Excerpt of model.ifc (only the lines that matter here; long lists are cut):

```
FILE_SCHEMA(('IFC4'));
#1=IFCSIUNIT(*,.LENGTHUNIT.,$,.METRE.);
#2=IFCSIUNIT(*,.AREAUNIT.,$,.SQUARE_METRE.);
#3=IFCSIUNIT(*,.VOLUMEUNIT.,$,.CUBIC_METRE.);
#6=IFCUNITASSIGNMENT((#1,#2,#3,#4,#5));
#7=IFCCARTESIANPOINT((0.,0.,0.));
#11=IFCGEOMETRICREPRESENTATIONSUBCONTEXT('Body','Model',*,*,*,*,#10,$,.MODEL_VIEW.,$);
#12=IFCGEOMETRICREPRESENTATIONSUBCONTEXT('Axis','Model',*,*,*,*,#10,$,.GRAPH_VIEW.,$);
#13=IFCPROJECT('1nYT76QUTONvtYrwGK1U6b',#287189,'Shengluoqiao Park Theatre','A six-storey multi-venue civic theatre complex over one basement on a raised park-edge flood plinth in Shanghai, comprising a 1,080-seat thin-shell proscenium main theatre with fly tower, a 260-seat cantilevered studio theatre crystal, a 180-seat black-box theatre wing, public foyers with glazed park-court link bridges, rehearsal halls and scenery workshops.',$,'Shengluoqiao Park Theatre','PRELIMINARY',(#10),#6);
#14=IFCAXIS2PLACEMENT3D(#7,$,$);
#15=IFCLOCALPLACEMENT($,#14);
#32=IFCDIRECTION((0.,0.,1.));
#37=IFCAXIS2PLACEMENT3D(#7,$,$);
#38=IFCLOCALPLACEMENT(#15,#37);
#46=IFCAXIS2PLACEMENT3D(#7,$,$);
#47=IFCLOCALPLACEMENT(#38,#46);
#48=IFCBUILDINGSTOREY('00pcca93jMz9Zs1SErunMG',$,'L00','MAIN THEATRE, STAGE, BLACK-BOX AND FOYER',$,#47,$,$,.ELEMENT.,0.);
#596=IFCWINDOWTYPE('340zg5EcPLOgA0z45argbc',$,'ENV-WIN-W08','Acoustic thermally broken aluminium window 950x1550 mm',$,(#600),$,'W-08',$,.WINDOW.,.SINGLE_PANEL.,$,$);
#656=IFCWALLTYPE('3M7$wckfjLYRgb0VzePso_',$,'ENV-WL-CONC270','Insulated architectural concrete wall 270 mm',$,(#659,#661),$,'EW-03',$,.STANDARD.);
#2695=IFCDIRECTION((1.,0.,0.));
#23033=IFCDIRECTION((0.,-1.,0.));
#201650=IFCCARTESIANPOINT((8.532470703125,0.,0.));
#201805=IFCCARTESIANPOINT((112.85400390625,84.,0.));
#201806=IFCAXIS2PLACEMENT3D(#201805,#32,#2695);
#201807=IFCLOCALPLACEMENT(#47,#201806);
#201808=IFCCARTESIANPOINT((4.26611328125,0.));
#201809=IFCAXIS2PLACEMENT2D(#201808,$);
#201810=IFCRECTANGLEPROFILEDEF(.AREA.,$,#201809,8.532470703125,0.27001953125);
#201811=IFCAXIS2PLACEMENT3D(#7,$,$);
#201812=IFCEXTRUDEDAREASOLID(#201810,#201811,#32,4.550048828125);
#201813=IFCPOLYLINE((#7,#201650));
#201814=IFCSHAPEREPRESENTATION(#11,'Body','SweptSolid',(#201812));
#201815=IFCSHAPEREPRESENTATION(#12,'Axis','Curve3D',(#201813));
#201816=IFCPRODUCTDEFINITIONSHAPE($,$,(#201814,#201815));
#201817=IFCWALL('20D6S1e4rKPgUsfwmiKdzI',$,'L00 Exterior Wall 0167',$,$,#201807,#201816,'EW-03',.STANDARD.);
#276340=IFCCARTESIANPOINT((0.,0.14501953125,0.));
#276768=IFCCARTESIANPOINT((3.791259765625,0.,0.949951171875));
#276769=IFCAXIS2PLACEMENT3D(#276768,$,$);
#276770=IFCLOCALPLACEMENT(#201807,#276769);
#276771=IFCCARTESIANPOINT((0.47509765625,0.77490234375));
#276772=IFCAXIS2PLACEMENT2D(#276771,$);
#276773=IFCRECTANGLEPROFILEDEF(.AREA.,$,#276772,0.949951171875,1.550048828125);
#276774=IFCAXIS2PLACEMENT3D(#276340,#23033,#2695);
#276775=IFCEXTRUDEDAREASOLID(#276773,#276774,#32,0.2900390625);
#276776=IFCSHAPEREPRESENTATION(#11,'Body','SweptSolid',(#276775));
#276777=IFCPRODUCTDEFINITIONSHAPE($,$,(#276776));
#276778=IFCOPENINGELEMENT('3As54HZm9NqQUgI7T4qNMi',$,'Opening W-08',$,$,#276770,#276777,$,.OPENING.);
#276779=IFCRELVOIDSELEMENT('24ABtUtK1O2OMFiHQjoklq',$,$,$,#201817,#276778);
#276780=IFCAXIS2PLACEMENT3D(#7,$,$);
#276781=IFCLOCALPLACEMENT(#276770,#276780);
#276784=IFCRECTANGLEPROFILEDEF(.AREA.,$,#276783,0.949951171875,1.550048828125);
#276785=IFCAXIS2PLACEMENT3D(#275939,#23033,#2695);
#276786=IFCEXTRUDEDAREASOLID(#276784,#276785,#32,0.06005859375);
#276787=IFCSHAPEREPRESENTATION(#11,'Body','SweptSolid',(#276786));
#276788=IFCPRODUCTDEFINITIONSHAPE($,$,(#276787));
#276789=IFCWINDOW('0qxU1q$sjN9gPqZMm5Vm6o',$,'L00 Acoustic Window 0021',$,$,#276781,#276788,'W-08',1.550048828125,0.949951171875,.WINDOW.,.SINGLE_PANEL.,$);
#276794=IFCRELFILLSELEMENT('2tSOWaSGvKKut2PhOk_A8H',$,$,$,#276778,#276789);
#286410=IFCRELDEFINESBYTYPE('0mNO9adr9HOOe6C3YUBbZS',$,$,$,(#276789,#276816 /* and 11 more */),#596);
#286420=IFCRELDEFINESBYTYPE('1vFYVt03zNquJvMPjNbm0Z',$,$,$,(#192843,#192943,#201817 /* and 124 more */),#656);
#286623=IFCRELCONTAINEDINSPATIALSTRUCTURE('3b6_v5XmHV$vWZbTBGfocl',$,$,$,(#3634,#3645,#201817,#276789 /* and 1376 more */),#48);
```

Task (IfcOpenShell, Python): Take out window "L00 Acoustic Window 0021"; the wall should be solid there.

```python
import ifcopenshell
import ifcopenshell.api.feature
import ifcopenshell.api.root
import ifcopenshell.geom
import ifcopenshell.util.shape

model = ifcopenshell.open("model.ifc")
settings = ifcopenshell.geom.settings()


def volume(element):
    """Net volume in cubic metres, openings subtracted."""
    shape = ifcopenshell.geom.create_shape(settings, element)
    return ifcopenshell.util.shape.get_volume(shape.geometry)


window = model.by_id(276789)
opening = window.FillsVoids[0].RelatingOpeningElement
wall = opening.VoidsElements[0].RelatingBuildingElement
before = volume(wall)

ifcopenshell.api.root.remove_product(model, product=window)
ifcopenshell.api.feature.remove_feature(model, feature=opening)

after = volume(wall)

print(f"wall volume {before:.3f} -> {after:.3f} m3")

model.write("model-out.ifc")
```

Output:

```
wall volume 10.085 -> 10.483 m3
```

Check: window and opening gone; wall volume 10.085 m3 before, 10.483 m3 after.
